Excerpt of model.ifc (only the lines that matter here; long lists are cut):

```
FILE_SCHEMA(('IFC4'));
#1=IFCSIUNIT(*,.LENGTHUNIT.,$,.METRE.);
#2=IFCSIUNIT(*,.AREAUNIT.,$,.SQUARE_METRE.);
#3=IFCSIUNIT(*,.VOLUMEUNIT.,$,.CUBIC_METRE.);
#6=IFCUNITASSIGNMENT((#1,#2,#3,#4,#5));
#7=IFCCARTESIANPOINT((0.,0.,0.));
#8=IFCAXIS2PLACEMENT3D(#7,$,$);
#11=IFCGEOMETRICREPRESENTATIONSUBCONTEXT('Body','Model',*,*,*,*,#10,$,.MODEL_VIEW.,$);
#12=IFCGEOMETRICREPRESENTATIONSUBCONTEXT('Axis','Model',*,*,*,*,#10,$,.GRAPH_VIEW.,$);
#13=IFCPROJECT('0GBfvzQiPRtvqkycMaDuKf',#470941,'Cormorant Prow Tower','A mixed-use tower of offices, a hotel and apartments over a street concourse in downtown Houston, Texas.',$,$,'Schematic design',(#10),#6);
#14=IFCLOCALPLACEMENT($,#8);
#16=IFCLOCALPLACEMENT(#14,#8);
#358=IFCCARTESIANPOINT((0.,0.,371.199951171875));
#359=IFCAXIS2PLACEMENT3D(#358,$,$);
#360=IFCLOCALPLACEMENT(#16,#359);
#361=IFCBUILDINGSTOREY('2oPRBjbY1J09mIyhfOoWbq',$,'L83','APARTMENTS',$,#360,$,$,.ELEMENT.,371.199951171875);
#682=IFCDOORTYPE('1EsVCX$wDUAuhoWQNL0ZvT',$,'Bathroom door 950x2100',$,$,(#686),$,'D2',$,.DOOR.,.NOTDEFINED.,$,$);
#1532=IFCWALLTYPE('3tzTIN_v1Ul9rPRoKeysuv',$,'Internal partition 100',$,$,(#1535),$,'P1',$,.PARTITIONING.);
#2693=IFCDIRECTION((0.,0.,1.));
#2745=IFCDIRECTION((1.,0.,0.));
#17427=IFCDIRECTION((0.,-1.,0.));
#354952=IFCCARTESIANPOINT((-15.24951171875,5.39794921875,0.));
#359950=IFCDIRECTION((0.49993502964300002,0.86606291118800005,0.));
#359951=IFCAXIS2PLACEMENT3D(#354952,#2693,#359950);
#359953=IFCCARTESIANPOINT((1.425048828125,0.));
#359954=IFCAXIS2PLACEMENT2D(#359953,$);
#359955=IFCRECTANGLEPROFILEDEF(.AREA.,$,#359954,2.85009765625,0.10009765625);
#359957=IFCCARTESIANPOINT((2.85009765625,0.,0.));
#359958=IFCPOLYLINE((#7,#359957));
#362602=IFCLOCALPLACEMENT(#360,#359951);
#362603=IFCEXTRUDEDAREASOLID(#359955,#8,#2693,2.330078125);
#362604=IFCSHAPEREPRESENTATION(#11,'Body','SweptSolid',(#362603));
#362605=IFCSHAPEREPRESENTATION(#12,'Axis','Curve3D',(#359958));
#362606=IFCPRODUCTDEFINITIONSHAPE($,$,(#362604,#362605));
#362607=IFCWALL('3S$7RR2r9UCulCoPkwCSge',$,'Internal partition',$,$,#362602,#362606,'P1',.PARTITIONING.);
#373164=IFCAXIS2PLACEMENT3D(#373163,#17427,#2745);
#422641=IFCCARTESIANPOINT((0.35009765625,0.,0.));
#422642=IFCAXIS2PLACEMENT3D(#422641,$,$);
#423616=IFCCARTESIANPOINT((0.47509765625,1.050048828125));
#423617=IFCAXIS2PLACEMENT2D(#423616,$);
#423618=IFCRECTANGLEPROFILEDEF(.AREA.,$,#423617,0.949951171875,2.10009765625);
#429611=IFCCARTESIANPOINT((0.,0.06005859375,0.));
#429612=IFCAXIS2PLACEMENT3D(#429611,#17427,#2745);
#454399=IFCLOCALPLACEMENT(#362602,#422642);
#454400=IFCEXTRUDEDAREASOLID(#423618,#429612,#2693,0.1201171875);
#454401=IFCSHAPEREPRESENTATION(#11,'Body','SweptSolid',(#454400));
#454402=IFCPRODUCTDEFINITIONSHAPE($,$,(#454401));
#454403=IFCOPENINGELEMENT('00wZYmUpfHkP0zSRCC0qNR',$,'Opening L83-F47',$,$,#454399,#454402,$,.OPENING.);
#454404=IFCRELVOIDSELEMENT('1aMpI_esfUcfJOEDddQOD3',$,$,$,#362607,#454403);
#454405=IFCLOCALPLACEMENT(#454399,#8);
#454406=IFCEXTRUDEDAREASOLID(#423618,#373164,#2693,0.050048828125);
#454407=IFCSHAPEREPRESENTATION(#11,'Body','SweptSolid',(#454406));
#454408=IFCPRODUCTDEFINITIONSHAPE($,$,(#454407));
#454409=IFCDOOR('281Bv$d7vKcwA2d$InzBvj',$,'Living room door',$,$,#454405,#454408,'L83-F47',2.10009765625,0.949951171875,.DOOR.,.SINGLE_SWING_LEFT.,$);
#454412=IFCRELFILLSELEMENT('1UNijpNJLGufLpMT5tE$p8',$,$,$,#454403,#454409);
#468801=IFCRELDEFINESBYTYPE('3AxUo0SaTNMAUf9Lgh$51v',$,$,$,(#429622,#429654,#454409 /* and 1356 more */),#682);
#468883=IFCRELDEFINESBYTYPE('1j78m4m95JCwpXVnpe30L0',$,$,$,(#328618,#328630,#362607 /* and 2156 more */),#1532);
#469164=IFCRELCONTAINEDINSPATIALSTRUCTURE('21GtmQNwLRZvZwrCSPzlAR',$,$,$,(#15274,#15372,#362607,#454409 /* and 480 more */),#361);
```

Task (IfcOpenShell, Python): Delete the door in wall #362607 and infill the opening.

```python
import ifcopenshell
import ifcopenshell.api.feature
import ifcopenshell.api.root
import ifcopenshell.geom
import ifcopenshell.util.shape

model = ifcopenshell.open("model.ifc")
settings = ifcopenshell.geom.settings()


def volume(element):
    """Net volume in cubic metres, openings subtracted."""
    shape = ifcopenshell.geom.create_shape(settings, element)
    return ifcopenshell.util.shape.get_volume(shape.geometry)


door = model.by_guid("281Bv$d7vKcwA2d$InzBvj")
opening = door.FillsVoids[0].RelatingOpeningElement
wall = opening.VoidsElements[0].RelatingBuildingElement
before = volume(wall)

ifcopenshell.api.root.remove_product(model, product=door)
ifcopenshell.api.feature.remove_feature(model, feature=opening)

after = volume(wall)

print(f"wall volume {before:.3f} -> {after:.3f} m3")

model.write("model_updated.ifc")
```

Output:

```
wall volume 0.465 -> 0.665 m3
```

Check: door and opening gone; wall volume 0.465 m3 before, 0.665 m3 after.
